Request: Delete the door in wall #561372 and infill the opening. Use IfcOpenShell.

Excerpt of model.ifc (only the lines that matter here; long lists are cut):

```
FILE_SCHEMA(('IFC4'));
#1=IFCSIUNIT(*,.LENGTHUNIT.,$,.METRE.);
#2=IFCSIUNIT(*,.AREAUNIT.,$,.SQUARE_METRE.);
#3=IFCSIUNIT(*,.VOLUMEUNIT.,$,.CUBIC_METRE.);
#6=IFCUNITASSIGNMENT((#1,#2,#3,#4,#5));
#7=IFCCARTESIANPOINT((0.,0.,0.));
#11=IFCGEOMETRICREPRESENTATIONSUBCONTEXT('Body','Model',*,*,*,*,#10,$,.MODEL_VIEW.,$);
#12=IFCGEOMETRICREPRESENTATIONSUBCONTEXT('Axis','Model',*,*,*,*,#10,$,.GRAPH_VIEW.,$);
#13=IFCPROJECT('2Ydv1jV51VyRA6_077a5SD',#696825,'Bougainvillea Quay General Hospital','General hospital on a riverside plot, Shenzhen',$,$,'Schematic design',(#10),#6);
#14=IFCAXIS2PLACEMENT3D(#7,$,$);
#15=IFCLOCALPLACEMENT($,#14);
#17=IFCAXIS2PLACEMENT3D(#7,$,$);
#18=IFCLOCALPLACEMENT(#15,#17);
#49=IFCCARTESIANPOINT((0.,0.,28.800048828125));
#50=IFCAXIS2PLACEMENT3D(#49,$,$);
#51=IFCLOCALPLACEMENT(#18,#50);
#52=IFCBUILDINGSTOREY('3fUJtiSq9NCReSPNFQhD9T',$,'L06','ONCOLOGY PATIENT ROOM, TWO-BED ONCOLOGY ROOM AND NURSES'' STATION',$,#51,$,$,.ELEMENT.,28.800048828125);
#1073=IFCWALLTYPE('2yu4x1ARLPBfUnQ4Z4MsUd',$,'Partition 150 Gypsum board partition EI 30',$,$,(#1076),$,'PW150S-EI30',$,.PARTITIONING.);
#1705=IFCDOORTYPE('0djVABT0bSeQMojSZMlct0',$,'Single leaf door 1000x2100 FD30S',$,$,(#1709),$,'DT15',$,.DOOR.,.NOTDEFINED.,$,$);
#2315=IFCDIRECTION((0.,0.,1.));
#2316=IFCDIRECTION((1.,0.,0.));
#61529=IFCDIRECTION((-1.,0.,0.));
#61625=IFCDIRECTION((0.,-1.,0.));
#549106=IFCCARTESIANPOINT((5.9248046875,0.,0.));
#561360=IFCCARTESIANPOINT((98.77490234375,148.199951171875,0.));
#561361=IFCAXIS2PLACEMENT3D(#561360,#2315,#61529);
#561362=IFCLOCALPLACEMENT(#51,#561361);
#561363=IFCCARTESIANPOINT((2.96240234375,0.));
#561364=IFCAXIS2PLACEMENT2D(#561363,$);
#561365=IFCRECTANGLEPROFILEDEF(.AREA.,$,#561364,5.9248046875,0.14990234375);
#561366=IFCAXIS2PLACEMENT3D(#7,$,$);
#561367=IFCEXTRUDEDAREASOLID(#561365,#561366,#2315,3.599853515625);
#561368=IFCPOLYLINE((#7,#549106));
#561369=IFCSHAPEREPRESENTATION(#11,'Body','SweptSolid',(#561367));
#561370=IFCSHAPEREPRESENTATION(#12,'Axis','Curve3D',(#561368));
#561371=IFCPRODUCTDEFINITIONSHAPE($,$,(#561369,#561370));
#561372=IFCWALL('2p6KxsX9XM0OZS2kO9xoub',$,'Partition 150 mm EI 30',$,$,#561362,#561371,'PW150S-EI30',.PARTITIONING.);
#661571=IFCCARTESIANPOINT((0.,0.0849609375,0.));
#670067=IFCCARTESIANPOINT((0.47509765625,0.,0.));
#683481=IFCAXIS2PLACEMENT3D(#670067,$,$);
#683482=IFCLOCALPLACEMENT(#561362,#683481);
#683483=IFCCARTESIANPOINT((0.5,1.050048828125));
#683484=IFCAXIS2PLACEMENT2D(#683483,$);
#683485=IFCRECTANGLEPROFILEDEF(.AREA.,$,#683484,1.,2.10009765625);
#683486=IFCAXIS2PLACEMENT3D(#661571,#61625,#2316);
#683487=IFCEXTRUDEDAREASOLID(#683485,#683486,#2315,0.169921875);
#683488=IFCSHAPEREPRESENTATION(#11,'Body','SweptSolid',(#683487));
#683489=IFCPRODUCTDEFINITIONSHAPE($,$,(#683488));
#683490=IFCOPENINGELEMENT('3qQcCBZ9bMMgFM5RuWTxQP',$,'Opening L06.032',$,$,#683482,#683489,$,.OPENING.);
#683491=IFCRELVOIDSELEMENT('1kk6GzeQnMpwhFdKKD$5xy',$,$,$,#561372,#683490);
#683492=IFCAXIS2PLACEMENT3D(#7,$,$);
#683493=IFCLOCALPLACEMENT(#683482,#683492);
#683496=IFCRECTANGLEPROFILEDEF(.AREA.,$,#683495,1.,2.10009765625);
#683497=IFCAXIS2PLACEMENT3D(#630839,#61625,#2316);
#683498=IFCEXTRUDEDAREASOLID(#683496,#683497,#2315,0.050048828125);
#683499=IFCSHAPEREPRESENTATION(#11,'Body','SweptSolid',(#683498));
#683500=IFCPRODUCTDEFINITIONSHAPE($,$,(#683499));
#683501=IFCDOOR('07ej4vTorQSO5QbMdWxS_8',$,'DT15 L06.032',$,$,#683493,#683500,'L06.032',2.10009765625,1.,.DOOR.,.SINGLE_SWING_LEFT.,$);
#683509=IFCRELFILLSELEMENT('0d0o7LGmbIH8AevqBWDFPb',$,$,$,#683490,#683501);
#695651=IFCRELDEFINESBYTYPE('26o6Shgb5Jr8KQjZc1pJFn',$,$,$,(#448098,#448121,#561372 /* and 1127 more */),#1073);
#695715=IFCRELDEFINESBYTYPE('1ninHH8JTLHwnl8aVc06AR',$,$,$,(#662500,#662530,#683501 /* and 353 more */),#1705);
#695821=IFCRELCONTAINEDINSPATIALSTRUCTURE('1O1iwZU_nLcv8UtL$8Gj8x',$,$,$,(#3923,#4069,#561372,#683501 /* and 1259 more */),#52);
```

```python
import ifcopenshell
import ifcopenshell.api.feature
import ifcopenshell.api.root
import ifcopenshell.geom
import ifcopenshell.util.shape

model = ifcopenshell.open("model.ifc")
settings = ifcopenshell.geom.settings()


def volume(element):
    """Net volume in cubic metres, openings subtracted."""
    shape = ifcopenshell.geom.create_shape(settings, element)
    return ifcopenshell.util.shape.get_volume(shape.geometry)


door = model.by_guid("07ej4vTorQSO5QbMdWxS_8")
opening = door.FillsVoids[0].RelatingOpeningElement
wall = opening.VoidsElements[0].RelatingBuildingElement
before = volume(wall)

ifcopenshell.api.root.remove_product(model, product=door)
ifcopenshell.api.feature.remove_feature(model, feature=opening)

after = volume(wall)

print(f"wall volume {before:.3f} -> {after:.3f} m3")

model.write("model_updated.ifc")
```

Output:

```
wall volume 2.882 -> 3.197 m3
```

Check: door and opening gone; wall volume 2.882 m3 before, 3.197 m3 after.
